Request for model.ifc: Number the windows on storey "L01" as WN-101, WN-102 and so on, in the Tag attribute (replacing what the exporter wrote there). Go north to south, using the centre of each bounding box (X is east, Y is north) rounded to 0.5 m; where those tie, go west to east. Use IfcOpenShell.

First a look at what the model holds.

```python
import ifcopenshell
import ifcopenshell.util.element
import ifcopenshell.util.placement

model = ifcopenshell.open("model.ifc")
print(model.schema)
storey = next(s for s in model.by_type("IfcBuildingStorey") if s.Name == "L01")
windows = [e for e in ifcopenshell.util.element.get_decomposition(storey) if e.is_a("IfcWindow")]
for e in sorted(windows, key=lambda e: e.id()):
    origin = ifcopenshell.util.placement.get_local_placement(e.ObjectPlacement)[:3, 3]
    print(e.id(), e.Tag, e.Name, origin.round(2) + 0.0, sep=" | ")
```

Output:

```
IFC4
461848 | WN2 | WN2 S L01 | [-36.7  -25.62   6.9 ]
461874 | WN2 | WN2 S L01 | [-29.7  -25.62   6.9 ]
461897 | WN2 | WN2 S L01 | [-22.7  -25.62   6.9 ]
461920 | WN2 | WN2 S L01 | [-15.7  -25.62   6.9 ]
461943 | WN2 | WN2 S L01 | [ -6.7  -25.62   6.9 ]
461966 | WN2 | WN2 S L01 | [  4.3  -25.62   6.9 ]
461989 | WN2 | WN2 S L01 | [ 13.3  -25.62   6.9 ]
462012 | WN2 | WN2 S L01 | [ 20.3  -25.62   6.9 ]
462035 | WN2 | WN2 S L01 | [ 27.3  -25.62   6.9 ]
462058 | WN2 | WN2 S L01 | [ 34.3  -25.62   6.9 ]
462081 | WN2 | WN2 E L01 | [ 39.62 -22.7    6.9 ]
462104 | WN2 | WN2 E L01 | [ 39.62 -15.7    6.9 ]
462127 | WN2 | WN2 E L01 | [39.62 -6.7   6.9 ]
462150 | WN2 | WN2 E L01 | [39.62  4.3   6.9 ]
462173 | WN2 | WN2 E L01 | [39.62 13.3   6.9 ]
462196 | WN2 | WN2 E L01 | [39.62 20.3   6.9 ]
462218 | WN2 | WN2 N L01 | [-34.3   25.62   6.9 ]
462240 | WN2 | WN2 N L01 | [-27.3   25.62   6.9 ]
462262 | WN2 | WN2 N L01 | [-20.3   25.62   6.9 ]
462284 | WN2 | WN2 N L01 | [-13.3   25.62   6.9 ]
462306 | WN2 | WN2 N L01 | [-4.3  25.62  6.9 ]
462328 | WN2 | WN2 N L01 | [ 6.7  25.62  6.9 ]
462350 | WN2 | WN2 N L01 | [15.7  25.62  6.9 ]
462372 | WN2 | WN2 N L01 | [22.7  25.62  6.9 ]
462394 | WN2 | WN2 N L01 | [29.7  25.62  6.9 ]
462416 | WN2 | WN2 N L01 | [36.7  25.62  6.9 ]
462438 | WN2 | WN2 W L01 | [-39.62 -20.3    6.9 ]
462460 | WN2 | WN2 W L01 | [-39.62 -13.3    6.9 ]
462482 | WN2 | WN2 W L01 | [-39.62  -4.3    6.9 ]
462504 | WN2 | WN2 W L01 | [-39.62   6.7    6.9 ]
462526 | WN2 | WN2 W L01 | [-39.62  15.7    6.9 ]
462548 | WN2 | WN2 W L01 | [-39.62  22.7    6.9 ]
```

```python
import ifcopenshell
import ifcopenshell.geom
import ifcopenshell.util.element
import ifcopenshell.util.shape

model = ifcopenshell.open("model.ifc")
settings = ifcopenshell.geom.settings()
settings.set("use-world-coords", True)


def centre(element):
    shape = ifcopenshell.geom.create_shape(settings, element)
    return ifcopenshell.util.shape.get_bbox_centroid(shape.geometry)


storey = next(s for s in model.by_type("IfcBuildingStorey") if s.Name == "L01")
windows = [e for e in ifcopenshell.util.element.get_decomposition(storey) if e.is_a("IfcWindow")]

# Insertion points can sit at a corner or the storey origin, so sort by the geometry (in metres).
centres = {e: centre(e) for e in windows}
windows.sort(key=lambda e: (-round(centres[e][1] / 0.5), centres[e][0]))

for i, e in enumerate(windows, start=1):
    number = f"WN-1{i:02d}"
    e.Tag = number
    print(e.id(), number)

model.write("model_edited.ifc")
```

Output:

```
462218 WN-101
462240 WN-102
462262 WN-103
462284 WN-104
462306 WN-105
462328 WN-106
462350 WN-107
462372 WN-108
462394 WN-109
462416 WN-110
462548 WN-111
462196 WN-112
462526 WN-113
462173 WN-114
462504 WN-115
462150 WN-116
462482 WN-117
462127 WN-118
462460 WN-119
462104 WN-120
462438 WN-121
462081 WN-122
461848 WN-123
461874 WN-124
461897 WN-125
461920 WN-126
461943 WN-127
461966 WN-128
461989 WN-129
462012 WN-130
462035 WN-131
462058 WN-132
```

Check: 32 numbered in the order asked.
